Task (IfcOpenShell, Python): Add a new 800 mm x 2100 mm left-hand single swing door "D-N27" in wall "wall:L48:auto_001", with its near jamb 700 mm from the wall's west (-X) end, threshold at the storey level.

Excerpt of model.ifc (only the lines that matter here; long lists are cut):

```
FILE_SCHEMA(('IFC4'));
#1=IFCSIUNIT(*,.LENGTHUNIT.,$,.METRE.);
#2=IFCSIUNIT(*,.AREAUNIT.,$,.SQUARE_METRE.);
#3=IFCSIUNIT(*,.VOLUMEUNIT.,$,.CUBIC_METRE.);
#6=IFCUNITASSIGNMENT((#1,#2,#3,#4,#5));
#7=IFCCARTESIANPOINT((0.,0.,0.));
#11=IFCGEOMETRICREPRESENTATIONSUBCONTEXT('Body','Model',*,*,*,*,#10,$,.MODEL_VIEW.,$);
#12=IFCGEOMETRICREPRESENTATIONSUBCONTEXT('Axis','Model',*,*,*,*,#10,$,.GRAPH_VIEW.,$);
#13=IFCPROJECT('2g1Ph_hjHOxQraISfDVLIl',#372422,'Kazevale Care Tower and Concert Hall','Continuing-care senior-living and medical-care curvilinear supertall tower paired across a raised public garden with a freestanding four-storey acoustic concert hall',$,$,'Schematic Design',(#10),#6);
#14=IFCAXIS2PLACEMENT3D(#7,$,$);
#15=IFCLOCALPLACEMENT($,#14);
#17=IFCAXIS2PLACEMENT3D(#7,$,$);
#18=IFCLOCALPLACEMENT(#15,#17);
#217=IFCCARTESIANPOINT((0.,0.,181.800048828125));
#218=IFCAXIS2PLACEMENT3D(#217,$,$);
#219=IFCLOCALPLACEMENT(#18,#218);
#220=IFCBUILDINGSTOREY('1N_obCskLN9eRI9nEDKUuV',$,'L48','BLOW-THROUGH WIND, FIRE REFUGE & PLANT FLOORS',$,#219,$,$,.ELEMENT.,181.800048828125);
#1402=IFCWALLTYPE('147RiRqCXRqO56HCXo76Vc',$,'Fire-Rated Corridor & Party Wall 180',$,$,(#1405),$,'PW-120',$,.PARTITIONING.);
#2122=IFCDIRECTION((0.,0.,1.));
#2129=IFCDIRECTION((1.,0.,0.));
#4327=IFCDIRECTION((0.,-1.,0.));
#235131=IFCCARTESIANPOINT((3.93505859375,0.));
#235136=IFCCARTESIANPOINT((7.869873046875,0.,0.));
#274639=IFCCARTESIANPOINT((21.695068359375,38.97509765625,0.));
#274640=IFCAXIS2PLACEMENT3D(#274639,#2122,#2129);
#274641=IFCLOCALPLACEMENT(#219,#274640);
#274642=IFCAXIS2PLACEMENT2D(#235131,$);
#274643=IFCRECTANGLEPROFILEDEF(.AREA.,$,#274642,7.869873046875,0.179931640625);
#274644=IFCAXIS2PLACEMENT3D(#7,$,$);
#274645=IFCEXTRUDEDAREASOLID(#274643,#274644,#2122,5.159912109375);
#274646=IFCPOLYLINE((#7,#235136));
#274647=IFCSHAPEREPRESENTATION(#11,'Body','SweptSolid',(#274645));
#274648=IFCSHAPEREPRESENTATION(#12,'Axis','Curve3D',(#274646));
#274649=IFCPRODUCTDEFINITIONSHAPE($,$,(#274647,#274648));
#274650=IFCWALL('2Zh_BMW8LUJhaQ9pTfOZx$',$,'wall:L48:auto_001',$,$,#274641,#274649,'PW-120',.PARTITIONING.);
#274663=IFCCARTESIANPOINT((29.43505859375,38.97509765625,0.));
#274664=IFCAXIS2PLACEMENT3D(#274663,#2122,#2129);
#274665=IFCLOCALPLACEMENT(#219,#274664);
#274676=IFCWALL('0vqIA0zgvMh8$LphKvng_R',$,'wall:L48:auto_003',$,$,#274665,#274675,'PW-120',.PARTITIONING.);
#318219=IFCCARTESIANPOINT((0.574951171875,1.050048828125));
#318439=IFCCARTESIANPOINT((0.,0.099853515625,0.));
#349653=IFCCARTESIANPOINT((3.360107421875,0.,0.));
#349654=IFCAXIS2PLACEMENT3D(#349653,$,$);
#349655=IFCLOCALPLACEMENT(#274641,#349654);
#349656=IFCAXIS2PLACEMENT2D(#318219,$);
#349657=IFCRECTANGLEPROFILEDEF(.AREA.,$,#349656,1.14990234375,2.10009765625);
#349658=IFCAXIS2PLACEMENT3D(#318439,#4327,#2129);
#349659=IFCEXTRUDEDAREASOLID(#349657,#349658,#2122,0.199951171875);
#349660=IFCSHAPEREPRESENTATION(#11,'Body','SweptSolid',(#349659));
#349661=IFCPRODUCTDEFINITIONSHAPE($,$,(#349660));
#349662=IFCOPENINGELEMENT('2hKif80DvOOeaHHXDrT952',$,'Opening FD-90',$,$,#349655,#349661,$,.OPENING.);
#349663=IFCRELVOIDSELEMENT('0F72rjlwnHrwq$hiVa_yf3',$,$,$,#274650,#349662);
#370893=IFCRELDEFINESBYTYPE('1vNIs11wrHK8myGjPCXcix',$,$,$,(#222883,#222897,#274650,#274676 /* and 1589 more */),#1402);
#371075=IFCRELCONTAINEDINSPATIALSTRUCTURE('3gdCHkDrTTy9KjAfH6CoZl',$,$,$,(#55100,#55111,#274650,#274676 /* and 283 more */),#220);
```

```python
import numpy as np
import ifcopenshell
import ifcopenshell.api.feature
import ifcopenshell.api.geometry
import ifcopenshell.api.root
import ifcopenshell.api.spatial
import ifcopenshell.geom
import ifcopenshell.util.element
import ifcopenshell.util.placement
import ifcopenshell.util.representation
import ifcopenshell.util.shape
import ifcopenshell.util.unit

model = ifcopenshell.open("model.ifc")
unit_scale = ifcopenshell.util.unit.calculate_unit_scale(model)
settings = ifcopenshell.geom.settings()


def volume(element):
    """Net volume in cubic metres, openings subtracted."""
    shape = ifcopenshell.geom.create_shape(settings, element)
    return ifcopenshell.util.shape.get_volume(shape.geometry)


wall = model.by_guid("2Zh_BMW8LUJhaQ9pTfOZx$")
storey = ifcopenshell.util.element.get_container(wall, ifc_class="IfcBuildingStorey")
context = ifcopenshell.util.representation.get_context(model, "Model", "Body", "MODEL_VIEW")
before = volume(wall)

width, height, from_end, sill = 0.8, 2.1, 0.7, 0.0  # metres

# The wall runs along its own X axis, and the end named is its -X end.
wall_shape = ifcopenshell.geom.create_shape(settings, wall)
x, y, z = ifcopenshell.util.shape.get_vertices(wall_shape.geometry).T
start = x.min() + from_end
face, thickness = float(y.min()), float(y.max() - y.min())
wall_matrix = ifcopenshell.util.placement.get_local_placement(wall.ObjectPlacement)
level = ifcopenshell.util.placement.get_local_placement(storey.ObjectPlacement)[2, 3]


def in_wall(x, y):
    """Placement at x, y metres in the wall's axes, at sill height."""
    matrix = wall_matrix.copy()
    matrix[:, 3] = wall_matrix @ np.array([x / unit_scale, y / unit_scale, 0.0, 1.0])
    matrix[2, 3] = level + sill / unit_scale
    return matrix


# Opening: a box that overshoots both wall faces by 50 mm.
opening = ifcopenshell.api.root.create_entity(model, ifc_class="IfcOpeningElement", predefined_type="OPENING")
box = ifcopenshell.api.geometry.add_wall_representation(
    model, context=context, length=width, height=height, thickness=thickness + 0.1
)
ifcopenshell.api.geometry.assign_representation(model, product=opening, representation=box)
ifcopenshell.api.geometry.edit_object_placement(model, product=opening, matrix=in_wall(start, face - 0.05), is_si=False)
ifcopenshell.api.feature.add_feature(model, feature=opening, element=wall)

door = ifcopenshell.api.root.create_entity(model, ifc_class="IfcDoor", name="D-N27", predefined_type="DOOR")
door.OverallWidth, door.OverallHeight = width / unit_scale, height / unit_scale
door.OperationType = "SINGLE_SWING_LEFT"
body = ifcopenshell.api.geometry.add_door_representation(
    model,
    context=context,
    overall_width=door.OverallWidth,
    overall_height=door.OverallHeight,
    operation_type="SINGLE_SWING_LEFT",
    lining_properties={"LiningDepth": thickness / unit_scale, "ThresholdDepth": thickness / unit_scale},
)
ifcopenshell.api.geometry.assign_representation(model, product=door, representation=body)
ifcopenshell.api.spatial.assign_container(model, products=[door], relating_structure=storey)
ifcopenshell.api.feature.add_filling(model, opening=opening, element=door)

# The lining spans the wall, so the door starts at the wall face.
ifcopenshell.api.geometry.edit_object_placement(model, product=door, matrix=in_wall(start, face), is_si=False)

after = volume(wall)

print(f"wall volume {before:.3f} -> {after:.3f} m3")

model.write("model_v2.ifc")
```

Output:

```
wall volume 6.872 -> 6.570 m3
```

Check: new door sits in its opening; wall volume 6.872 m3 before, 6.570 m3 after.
